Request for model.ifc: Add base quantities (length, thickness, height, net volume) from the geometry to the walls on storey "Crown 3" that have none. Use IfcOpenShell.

First a look at what the model holds.

```python
import ifcopenshell
import ifcopenshell.util.element
import ifcopenshell.util.unit

model = ifcopenshell.open("model.ifc")
print(model.schema)
for unit_type in ("LENGTHUNIT", "AREAUNIT", "VOLUMEUNIT"):
    print(unit_type, ifcopenshell.util.unit.calculate_unit_scale(model, unit_type))
storey = next(s for s in model.by_type("IfcBuildingStorey") if s.Name == "Crown 3")
walls = [e for e in ifcopenshell.util.element.get_decomposition(storey) if e.is_a("IfcWall")]
for e in sorted(walls, key=lambda e: e.id()):
    print(e.id(), e.is_a(), e.Name, list(ifcopenshell.util.element.get_psets(e, qtos_only=True)), sep=" | ")
```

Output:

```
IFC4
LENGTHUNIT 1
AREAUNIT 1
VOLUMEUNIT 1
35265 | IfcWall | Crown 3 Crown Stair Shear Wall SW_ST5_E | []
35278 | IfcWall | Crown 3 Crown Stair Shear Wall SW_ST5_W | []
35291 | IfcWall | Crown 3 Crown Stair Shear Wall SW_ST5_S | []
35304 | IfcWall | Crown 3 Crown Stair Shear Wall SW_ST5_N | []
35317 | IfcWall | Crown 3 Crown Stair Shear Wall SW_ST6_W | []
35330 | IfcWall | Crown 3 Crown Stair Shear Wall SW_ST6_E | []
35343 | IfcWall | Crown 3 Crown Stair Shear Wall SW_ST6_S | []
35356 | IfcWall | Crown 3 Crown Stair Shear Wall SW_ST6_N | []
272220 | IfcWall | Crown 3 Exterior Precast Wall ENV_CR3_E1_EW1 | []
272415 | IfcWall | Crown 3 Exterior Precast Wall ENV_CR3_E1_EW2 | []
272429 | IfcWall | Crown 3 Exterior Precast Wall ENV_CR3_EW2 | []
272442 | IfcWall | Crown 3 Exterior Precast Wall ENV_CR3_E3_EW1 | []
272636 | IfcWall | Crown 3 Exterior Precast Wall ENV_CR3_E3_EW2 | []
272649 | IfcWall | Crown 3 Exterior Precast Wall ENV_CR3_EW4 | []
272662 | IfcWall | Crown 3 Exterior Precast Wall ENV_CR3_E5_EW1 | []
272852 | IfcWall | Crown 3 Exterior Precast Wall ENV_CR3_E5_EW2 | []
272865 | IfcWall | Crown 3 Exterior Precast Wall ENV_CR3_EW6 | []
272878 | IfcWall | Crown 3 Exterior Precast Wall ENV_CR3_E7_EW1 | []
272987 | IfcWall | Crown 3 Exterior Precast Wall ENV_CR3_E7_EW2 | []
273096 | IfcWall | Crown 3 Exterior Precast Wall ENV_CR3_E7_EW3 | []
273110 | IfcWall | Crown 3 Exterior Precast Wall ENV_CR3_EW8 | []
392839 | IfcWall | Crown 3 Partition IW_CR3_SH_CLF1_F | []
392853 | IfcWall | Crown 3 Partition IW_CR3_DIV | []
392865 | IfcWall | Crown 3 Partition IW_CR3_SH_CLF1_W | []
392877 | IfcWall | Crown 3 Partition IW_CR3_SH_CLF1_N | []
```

```python
import ifcopenshell
import ifcopenshell.api.pset
import ifcopenshell.geom
import ifcopenshell.util.element
import ifcopenshell.util.shape
import ifcopenshell.util.unit

model = ifcopenshell.open("model.ifc")
unit_scale = ifcopenshell.util.unit.calculate_unit_scale(model)
volume_scale = ifcopenshell.util.unit.calculate_unit_scale(model, "VOLUMEUNIT")
settings = ifcopenshell.geom.settings()

storey = next(s for s in model.by_type("IfcBuildingStorey") if s.Name == "Crown 3")
walls = [e for e in ifcopenshell.util.element.get_decomposition(storey) if e.is_a("IfcWall")]

for e in sorted(walls, key=lambda e: e.id()):
    if ifcopenshell.util.element.get_psets(e, qtos_only=True, should_inherit=False):
        continue
    # Geometry comes back in metres, in the element's own axes.
    shape = ifcopenshell.geom.create_shape(settings, e)
    values = {
        "Length": ifcopenshell.util.shape.get_x(shape.geometry) / unit_scale,
        "Width": ifcopenshell.util.shape.get_y(shape.geometry) / unit_scale,
        "Height": ifcopenshell.util.shape.get_z(shape.geometry) / unit_scale,
        "NetVolume": ifcopenshell.util.shape.get_volume(shape.geometry) / volume_scale,
    }
    qto = ifcopenshell.api.pset.add_qto(model, product=e, name="Qto_WallBaseQuantities")
    ifcopenshell.api.pset.edit_qto(model, qto=qto, properties=values)
    print(e.id(), {k: round(v, 3) for k, v in values.items()})

model.write("model_v2.ifc")
```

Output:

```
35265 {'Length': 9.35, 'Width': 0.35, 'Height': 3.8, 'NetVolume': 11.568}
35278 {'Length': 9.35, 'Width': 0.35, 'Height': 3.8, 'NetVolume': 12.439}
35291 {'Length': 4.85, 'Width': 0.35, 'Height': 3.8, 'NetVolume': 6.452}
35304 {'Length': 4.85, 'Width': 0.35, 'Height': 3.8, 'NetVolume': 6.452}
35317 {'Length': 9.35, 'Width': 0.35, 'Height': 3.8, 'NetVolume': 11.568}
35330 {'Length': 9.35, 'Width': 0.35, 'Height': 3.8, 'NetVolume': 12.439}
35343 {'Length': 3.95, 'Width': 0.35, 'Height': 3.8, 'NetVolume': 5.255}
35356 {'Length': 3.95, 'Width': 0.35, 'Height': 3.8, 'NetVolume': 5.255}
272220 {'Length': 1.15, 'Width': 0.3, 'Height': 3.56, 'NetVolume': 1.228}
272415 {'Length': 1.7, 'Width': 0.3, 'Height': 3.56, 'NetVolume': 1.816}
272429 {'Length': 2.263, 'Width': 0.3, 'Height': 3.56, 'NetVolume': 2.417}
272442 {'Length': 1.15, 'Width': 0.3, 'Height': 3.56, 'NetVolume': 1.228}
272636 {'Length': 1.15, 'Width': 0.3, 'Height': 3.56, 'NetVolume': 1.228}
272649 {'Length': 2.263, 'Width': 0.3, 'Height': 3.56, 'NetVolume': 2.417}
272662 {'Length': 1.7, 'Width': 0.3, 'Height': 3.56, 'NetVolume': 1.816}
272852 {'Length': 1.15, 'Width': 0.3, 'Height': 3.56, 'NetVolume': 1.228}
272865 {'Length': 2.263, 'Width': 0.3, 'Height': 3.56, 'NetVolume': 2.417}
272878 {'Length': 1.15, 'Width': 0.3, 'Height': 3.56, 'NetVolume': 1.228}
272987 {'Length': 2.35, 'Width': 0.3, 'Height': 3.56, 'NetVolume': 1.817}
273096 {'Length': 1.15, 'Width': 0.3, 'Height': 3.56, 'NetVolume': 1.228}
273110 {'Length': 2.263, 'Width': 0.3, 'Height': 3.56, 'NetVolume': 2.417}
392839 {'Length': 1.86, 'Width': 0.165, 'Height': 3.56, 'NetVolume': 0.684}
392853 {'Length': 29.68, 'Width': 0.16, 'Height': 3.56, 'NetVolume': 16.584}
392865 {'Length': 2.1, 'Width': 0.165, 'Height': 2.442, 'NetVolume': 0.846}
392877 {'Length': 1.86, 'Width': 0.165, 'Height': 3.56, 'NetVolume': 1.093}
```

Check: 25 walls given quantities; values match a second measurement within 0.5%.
